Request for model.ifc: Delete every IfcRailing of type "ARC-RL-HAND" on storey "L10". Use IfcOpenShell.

First a look at what the model holds.

```python
import ifcopenshell
import ifcopenshell.util.element

model = ifcopenshell.open("model.ifc")
print(model.schema)
storey = next(s for s in model.by_type("IfcBuildingStorey") if s.Name == "L10")
railings = [e for e in ifcopenshell.util.element.get_decomposition(storey) if e.is_a("IfcRailing")]
seen = {}
for e in railings:
    element_type = ifcopenshell.util.element.get_type(e)
    name = element_type.Name if element_type not in (None, e) else None
    seen[name] = seen.get(name, 0) + 1
for name, count in sorted(seen.items(), key=str):
    print(count, "x", name)
```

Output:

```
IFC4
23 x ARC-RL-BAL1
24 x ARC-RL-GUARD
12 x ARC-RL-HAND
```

```python
import ifcopenshell
import ifcopenshell.api.root
import ifcopenshell.util.element

model = ifcopenshell.open("model.ifc")

storey = next(s for s in model.by_type("IfcBuildingStorey") if s.Name == "L10")
railings = [e for e in ifcopenshell.util.element.get_decomposition(storey) if e.is_a("IfcRailing")]
targets = [e for e in railings if (t := ifcopenshell.util.element.get_type(e)) not in (None, e) and t.Name == "ARC-RL-HAND"]

for e in targets:
    ifcopenshell.api.root.remove_product(model, product=e)
print(len(targets), "removed")

model.write("model_edited.ifc")
```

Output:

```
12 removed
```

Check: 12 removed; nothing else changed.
